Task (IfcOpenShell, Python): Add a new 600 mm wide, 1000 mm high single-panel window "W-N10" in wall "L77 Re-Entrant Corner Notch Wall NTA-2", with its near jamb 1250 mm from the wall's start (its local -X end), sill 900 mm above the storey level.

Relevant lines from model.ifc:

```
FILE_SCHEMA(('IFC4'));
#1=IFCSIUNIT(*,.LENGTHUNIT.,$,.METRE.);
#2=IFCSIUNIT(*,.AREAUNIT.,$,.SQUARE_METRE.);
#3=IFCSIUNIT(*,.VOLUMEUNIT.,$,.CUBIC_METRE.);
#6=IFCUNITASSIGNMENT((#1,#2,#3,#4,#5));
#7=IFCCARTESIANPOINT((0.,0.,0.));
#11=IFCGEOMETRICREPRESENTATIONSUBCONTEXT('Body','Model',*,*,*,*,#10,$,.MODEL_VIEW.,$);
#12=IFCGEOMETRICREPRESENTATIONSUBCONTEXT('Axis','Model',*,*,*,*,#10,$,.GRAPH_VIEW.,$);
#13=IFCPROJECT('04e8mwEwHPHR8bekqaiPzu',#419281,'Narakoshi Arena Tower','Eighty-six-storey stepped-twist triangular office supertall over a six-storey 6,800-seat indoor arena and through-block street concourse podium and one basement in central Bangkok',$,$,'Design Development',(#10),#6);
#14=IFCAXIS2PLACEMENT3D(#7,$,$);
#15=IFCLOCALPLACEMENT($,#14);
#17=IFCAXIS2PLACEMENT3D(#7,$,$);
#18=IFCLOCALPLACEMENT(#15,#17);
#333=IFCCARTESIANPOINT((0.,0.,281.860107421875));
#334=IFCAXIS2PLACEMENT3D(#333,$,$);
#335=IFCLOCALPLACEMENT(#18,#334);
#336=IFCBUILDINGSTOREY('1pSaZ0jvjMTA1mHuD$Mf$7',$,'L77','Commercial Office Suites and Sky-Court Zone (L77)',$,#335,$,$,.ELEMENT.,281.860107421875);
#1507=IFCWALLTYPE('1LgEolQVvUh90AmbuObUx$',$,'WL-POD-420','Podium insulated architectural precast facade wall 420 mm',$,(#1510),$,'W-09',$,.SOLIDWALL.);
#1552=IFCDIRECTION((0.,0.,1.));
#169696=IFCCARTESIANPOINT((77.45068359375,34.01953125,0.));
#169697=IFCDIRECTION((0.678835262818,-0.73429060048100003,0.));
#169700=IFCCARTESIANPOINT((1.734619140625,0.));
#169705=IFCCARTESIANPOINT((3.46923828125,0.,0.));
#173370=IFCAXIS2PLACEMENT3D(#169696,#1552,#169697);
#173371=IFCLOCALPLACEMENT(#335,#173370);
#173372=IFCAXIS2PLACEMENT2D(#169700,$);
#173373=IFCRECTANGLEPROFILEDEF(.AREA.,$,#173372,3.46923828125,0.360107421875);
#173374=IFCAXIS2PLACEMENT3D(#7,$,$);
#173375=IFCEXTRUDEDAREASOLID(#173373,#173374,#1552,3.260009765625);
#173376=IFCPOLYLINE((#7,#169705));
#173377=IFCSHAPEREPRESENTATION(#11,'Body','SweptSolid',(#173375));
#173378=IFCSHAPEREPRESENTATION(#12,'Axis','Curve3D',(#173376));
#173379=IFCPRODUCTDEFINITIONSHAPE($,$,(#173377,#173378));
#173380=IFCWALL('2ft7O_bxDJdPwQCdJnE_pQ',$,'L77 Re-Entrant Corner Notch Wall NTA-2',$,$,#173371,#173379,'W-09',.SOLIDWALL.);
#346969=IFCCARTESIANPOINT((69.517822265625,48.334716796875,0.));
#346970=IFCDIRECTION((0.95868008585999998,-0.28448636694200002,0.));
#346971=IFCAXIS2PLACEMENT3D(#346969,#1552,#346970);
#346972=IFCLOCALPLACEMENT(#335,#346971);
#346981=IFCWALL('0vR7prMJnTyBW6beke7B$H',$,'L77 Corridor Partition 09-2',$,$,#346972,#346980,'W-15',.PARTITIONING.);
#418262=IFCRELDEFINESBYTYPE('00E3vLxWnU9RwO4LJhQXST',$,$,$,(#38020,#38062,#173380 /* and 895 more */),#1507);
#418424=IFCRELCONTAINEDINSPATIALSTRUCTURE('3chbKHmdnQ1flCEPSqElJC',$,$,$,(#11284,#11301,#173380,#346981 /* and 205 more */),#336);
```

```python
import numpy as np
import ifcopenshell
import ifcopenshell.api.feature
import ifcopenshell.api.geometry
import ifcopenshell.api.root
import ifcopenshell.api.spatial
import ifcopenshell.geom
import ifcopenshell.util.element
import ifcopenshell.util.placement
import ifcopenshell.util.representation
import ifcopenshell.util.shape
import ifcopenshell.util.unit

model = ifcopenshell.open("model.ifc")
unit_scale = ifcopenshell.util.unit.calculate_unit_scale(model)
settings = ifcopenshell.geom.settings()


def volume(element):
    """Net volume in cubic metres, openings subtracted."""
    shape = ifcopenshell.geom.create_shape(settings, element)
    return ifcopenshell.util.shape.get_volume(shape.geometry)


wall = model.by_id(173380)
storey = ifcopenshell.util.element.get_container(wall, ifc_class="IfcBuildingStorey")
context = ifcopenshell.util.representation.get_context(model, "Model", "Body", "MODEL_VIEW")
before = volume(wall)

width, height, from_end, sill = 0.6, 1, 1.25, 0.9  # metres

# The wall runs along its own X axis, and the end named is its -X end.
wall_shape = ifcopenshell.geom.create_shape(settings, wall)
x, y, z = ifcopenshell.util.shape.get_vertices(wall_shape.geometry).T
start = x.min() + from_end
face, thickness = float(y.min()), float(y.max() - y.min())
wall_matrix = ifcopenshell.util.placement.get_local_placement(wall.ObjectPlacement)
level = ifcopenshell.util.placement.get_local_placement(storey.ObjectPlacement)[2, 3]


def in_wall(x, y):
    """Placement at x, y metres in the wall's axes, at sill height."""
    matrix = wall_matrix.copy()
    matrix[:, 3] = wall_matrix @ np.array([x / unit_scale, y / unit_scale, 0.0, 1.0])
    matrix[2, 3] = level + sill / unit_scale
    return matrix


# Opening: a box that overshoots both wall faces by 50 mm.
opening = ifcopenshell.api.root.create_entity(model, ifc_class="IfcOpeningElement", predefined_type="OPENING")
box = ifcopenshell.api.geometry.add_wall_representation(
    model, context=context, length=width, height=height, thickness=thickness + 0.1
)
ifcopenshell.api.geometry.assign_representation(model, product=opening, representation=box)
ifcopenshell.api.geometry.edit_object_placement(model, product=opening, matrix=in_wall(start, face - 0.05), is_si=False)
ifcopenshell.api.feature.add_feature(model, feature=opening, element=wall)

window = ifcopenshell.api.root.create_entity(model, ifc_class="IfcWindow", name="W-N10", predefined_type="WINDOW")
window.OverallWidth, window.OverallHeight = width / unit_scale, height / unit_scale
window.PartitioningType = "SINGLE_PANEL"
body = ifcopenshell.api.geometry.add_window_representation(
    model,
    context=context,
    overall_width=window.OverallWidth,
    overall_height=window.OverallHeight,
    partition_type="SINGLE_PANEL",
)
ifcopenshell.api.geometry.assign_representation(model, product=window, representation=body)
ifcopenshell.api.spatial.assign_container(model, products=[window], relating_structure=storey)
ifcopenshell.api.feature.add_filling(model, opening=opening, element=window)

# Centre the window in the wall's thickness.
ifcopenshell.api.geometry.edit_object_placement(model, product=window, matrix=in_wall(start, face), is_si=False)
window_shape = ifcopenshell.geom.create_shape(settings, window)
depth = ifcopenshell.util.shape.get_vertices(window_shape.geometry)[:, 1]
offset = face + thickness / 2 - (depth.min() + depth.max()) / 2
ifcopenshell.api.geometry.edit_object_placement(model, product=window, matrix=in_wall(start, offset), is_si=False)

after = volume(wall)

print(f"wall volume {before:.3f} -> {after:.3f} m3")

model.write("model_updated.ifc")
```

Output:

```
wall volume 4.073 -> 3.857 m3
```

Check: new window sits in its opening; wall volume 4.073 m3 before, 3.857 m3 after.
